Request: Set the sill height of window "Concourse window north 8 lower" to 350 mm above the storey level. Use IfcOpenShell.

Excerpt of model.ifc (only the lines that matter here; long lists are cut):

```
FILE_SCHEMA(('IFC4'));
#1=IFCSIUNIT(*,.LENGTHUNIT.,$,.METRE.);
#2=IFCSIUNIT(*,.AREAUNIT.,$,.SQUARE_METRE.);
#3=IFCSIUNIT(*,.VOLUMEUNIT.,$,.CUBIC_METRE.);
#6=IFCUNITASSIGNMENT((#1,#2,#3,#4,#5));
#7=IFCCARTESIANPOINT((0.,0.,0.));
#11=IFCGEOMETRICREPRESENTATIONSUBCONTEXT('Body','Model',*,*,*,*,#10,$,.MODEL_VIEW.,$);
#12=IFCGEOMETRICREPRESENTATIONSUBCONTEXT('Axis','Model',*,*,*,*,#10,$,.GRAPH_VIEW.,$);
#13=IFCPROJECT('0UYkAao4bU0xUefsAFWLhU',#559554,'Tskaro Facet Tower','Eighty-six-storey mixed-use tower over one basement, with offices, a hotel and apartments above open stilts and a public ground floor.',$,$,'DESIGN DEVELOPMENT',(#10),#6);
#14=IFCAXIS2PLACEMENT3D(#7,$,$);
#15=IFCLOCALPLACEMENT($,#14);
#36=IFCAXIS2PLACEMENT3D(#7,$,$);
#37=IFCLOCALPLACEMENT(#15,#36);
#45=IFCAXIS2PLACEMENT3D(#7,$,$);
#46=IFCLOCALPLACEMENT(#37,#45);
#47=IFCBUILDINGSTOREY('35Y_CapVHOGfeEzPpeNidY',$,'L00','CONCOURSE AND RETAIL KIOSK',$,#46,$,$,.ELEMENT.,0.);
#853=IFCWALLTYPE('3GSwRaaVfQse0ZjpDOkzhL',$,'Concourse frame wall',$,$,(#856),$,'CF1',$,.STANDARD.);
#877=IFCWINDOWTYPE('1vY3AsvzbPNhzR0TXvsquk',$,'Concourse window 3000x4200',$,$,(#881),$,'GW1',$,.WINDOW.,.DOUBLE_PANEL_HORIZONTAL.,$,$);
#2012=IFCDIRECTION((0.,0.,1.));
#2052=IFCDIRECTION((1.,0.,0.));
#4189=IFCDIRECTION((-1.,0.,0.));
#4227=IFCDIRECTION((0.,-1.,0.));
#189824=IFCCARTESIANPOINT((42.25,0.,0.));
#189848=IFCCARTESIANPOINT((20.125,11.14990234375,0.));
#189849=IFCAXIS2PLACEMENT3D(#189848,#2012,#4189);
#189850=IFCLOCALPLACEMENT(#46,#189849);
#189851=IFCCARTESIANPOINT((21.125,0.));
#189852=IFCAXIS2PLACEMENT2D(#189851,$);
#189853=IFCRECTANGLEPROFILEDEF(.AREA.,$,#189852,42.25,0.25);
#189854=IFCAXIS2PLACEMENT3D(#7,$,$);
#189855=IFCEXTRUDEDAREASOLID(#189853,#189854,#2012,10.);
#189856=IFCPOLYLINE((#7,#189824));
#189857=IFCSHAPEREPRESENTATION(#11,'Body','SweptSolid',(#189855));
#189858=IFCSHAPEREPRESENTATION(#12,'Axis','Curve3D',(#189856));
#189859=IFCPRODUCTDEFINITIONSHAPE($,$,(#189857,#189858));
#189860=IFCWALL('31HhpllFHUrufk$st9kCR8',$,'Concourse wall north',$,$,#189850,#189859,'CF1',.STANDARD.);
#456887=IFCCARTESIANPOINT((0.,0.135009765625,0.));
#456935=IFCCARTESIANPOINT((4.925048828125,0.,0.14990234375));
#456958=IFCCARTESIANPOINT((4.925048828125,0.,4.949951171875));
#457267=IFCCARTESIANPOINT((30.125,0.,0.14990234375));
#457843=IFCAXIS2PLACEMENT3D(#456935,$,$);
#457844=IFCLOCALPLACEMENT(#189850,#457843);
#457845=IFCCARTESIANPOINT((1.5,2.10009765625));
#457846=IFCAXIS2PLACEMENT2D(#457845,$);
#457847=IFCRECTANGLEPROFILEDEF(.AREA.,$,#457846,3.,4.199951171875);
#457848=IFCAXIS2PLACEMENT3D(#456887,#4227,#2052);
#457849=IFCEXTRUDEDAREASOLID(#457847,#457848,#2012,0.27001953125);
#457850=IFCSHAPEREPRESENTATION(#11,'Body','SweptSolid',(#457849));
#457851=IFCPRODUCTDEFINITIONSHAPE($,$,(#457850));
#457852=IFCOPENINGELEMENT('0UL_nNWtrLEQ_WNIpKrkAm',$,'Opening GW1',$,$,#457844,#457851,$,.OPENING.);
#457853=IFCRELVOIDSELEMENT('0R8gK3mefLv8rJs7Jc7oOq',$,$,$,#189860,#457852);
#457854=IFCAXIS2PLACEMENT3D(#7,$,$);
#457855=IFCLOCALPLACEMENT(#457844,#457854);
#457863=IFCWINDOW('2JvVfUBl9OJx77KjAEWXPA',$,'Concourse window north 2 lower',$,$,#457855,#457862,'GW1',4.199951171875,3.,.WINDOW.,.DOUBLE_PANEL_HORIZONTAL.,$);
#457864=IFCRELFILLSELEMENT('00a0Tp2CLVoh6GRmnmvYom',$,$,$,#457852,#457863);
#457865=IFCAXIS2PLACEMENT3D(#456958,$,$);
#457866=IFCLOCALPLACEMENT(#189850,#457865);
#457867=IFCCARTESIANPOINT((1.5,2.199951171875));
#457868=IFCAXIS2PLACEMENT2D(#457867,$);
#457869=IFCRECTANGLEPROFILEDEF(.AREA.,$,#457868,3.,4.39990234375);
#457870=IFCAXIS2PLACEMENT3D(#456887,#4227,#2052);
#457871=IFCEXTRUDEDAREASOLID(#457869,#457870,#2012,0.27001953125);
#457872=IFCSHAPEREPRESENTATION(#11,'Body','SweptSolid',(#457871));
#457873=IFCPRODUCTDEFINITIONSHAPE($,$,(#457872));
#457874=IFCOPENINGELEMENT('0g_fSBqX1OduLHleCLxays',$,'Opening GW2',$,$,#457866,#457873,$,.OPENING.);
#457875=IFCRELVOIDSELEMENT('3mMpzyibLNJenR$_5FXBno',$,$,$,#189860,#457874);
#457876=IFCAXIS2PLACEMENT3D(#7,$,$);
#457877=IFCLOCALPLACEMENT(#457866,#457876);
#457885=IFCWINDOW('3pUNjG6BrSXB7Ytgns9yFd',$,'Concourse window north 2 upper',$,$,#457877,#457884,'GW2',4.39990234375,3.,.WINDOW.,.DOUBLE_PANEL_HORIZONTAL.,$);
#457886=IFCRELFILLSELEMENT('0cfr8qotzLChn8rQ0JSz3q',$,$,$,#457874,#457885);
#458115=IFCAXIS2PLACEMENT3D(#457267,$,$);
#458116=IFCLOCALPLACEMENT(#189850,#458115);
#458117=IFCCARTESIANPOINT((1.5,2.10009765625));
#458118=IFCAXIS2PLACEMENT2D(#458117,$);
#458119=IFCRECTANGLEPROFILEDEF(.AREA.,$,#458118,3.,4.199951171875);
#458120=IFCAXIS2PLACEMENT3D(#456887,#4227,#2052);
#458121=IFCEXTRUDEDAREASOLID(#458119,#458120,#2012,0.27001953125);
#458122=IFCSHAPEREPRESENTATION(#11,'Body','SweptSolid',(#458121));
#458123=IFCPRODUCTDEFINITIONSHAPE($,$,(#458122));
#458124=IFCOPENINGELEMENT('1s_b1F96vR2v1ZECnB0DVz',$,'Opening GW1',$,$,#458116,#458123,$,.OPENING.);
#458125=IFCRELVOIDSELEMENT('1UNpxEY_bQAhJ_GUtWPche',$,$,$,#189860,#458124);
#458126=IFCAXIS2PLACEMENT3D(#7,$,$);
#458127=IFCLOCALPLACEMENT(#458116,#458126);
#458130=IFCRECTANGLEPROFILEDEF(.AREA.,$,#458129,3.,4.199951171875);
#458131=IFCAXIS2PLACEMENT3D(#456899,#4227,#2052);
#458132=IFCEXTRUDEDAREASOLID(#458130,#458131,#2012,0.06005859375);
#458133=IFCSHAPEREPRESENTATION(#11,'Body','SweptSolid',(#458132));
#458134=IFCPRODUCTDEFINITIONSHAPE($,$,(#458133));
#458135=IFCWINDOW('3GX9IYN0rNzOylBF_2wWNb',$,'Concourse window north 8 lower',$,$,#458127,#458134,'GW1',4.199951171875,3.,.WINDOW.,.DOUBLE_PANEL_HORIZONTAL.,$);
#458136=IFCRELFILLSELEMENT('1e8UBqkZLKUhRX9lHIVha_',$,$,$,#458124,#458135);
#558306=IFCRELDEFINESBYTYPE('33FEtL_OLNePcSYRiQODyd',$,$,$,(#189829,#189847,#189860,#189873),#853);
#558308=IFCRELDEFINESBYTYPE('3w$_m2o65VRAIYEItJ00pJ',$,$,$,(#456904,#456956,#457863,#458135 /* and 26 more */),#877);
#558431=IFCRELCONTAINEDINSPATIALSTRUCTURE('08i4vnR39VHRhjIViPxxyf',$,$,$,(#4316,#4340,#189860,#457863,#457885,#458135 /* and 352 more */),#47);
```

```python
import numpy as np
import ifcopenshell
import ifcopenshell.api.geometry
import ifcopenshell.geom
import ifcopenshell.util.element
import ifcopenshell.util.placement
import ifcopenshell.util.shape
import ifcopenshell.util.unit

model = ifcopenshell.open("model.ifc")
unit_scale = ifcopenshell.util.unit.calculate_unit_scale(model)

window = model.by_id(458135)
opening = window.FillsVoids[0].RelatingOpeningElement
storey = ifcopenshell.util.element.get_container(window, ifc_class="IfcBuildingStorey")
level = ifcopenshell.util.placement.get_local_placement(storey.ObjectPlacement)[2, 3]

# The opening's origin need not be at the sill, so measure its lowest point.
shape = ifcopenshell.geom.create_shape(ifcopenshell.geom.settings(), opening)
bottom = ifcopenshell.util.shape.get_shape_bottom_elevation(shape, shape.geometry) / unit_scale
dz = level + 0.35 / unit_scale - bottom

shift = np.array([0.0, 0.0, dz])
# The window is placed relative to its opening, so it follows when the opening moves.
matrix = ifcopenshell.util.placement.get_local_placement(opening.ObjectPlacement)
matrix[:3, 3] += shift
ifcopenshell.api.geometry.edit_object_placement(
    model, product=opening, matrix=matrix, is_si=False, should_transform_children=True
)

print(f"moved by {dz * unit_scale:+.3f} m")

model.write("model-out.ifc")
```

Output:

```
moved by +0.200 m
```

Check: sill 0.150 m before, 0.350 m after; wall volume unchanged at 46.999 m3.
